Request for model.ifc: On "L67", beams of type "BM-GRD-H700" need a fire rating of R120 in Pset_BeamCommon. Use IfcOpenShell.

First a look at what the model holds.

```python
import ifcopenshell
import ifcopenshell.util.element

model = ifcopenshell.open("model.ifc")
print(model.schema)
storey = next(s for s in model.by_type("IfcBuildingStorey") if s.Name == "L67")
beams = [e for e in ifcopenshell.util.element.get_decomposition(storey) if e.is_a("IfcBeam")]
seen = {}
for e in beams:
    element_type = ifcopenshell.util.element.get_type(e)
    key = (element_type.Name if element_type != e and element_type else None, ifcopenshell.util.element.get_pset(e, "Pset_BeamCommon", "FireRating"))
    seen[key] = seen.get(key, 0) + 1
for (name, value), count in sorted(seen.items(), key=str):
    print(count, "x", name, "|", value)
```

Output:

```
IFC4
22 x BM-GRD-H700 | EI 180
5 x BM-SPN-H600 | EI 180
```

```python
import ifcopenshell
import ifcopenshell.api.pset
import ifcopenshell.util.element

model = ifcopenshell.open("model.ifc")

storey = next(s for s in model.by_type("IfcBuildingStorey") if s.Name == "L67")
beams = [e for e in ifcopenshell.util.element.get_decomposition(storey) if e.is_a("IfcBeam")]

count = 0
for e in beams:
    element_type = ifcopenshell.util.element.get_type(e)
    if element_type in (None, e) or element_type.Name != "BM-GRD-H700":
        continue
    # add_pset returns the element's existing set when there is one.
    pset = ifcopenshell.api.pset.add_pset(model, product=e, name="Pset_BeamCommon")
    ifcopenshell.api.pset.edit_pset(model, pset=pset, properties={"FireRating": "R120"})
    count += 1

print(count, "beams updated")

model.write("model_updated.ifc")
```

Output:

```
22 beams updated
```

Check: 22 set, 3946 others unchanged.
